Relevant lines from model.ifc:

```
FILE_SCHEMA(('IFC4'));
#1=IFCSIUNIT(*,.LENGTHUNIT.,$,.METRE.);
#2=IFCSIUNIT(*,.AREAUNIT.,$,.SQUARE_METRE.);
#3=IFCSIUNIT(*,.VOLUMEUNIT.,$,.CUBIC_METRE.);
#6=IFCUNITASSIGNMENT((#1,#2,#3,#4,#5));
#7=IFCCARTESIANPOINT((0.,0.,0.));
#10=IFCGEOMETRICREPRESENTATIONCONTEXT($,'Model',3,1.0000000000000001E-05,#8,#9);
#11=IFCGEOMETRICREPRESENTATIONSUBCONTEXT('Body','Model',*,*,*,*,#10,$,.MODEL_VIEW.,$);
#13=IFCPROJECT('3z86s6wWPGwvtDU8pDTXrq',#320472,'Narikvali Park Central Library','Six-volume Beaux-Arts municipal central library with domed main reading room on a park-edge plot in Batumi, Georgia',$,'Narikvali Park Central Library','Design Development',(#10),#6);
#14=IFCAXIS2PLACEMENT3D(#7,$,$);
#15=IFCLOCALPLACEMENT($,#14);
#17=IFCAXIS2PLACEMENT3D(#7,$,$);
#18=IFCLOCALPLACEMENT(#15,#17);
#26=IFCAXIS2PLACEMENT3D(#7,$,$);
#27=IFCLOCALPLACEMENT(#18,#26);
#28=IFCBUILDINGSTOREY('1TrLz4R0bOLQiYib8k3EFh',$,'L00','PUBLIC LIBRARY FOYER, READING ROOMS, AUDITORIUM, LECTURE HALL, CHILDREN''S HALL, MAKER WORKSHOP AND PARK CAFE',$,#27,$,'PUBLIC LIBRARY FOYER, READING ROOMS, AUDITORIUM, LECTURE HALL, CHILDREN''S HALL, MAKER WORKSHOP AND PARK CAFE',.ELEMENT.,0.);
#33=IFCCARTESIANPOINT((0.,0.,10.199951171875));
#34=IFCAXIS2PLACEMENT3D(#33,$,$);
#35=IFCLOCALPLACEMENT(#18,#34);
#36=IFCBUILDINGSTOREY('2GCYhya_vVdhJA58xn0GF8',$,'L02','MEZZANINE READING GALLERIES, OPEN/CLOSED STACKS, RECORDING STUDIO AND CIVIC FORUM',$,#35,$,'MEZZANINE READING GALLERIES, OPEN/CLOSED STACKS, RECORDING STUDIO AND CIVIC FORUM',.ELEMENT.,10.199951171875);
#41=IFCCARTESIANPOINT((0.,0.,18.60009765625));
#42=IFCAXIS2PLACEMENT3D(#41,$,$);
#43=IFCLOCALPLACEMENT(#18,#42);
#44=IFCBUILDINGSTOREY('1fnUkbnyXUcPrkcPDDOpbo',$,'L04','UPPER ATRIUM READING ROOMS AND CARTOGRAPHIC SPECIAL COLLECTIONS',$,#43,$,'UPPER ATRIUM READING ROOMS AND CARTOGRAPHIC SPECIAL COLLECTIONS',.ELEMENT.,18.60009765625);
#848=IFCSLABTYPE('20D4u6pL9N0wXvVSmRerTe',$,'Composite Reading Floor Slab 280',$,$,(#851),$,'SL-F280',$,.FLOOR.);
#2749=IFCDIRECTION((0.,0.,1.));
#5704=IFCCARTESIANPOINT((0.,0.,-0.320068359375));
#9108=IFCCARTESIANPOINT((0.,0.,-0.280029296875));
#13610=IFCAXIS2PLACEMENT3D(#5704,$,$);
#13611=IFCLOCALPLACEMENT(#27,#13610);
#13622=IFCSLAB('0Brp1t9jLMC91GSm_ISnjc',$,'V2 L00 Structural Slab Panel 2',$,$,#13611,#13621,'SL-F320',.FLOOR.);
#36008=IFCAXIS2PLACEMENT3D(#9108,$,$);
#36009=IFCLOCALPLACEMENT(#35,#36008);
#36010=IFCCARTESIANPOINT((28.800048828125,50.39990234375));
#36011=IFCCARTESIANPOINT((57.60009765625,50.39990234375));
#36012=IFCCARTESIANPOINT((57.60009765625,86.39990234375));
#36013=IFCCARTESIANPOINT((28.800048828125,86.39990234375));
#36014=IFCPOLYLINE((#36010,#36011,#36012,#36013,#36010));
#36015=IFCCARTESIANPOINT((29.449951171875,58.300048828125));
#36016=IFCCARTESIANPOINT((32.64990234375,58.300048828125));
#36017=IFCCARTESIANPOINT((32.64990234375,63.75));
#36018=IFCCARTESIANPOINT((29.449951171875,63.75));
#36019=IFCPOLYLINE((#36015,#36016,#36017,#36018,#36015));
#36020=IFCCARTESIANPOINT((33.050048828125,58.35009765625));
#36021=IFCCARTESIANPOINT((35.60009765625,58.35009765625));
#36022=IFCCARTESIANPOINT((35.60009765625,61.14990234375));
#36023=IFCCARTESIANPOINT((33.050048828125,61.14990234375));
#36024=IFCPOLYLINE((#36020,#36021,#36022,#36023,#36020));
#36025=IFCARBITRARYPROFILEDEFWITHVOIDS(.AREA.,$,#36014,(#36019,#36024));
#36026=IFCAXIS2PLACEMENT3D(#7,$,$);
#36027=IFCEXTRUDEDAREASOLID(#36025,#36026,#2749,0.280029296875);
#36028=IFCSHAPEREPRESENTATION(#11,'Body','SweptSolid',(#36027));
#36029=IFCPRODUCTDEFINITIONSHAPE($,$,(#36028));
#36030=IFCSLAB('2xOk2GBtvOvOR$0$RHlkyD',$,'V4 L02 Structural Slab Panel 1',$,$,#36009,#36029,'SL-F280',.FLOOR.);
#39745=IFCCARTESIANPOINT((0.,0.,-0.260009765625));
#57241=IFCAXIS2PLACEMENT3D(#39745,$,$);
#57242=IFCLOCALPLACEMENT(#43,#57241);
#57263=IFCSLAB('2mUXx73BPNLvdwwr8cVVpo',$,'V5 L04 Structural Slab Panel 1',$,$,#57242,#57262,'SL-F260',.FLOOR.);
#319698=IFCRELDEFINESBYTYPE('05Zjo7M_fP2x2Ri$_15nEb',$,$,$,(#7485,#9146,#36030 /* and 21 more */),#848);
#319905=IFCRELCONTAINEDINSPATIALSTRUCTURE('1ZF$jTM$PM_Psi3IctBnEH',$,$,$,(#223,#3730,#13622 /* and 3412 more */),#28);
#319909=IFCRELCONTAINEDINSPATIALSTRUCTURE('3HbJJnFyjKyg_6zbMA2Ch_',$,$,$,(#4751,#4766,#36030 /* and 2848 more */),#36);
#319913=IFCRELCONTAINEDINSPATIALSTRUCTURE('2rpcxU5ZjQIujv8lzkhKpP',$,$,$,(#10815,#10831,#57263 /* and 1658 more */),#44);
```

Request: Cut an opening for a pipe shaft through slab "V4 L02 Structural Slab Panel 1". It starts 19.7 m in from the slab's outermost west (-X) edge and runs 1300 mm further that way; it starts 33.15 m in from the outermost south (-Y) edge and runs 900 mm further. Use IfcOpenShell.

```python
import numpy as np
import ifcopenshell
import ifcopenshell.api.feature
import ifcopenshell.api.geometry
import ifcopenshell.api.root
import ifcopenshell.geom
import ifcopenshell.util.placement
import ifcopenshell.util.representation
import ifcopenshell.util.shape
import ifcopenshell.util.unit

model = ifcopenshell.open("model.ifc")
unit_scale = ifcopenshell.util.unit.calculate_unit_scale(model)
settings = ifcopenshell.geom.settings()


def volume(element):
    """Net volume in cubic metres, openings subtracted."""
    shape = ifcopenshell.geom.create_shape(settings, element)
    return ifcopenshell.util.shape.get_volume(shape.geometry)


slab = model.by_guid("2xOk2GBtvOvOR$0$RHlkyD")
before = volume(slab)

# Extent in the slab's own axes, in metres. The edges named are its -X and -Y sides.
slab_shape = ifcopenshell.geom.create_shape(settings, slab)
vertices = ifcopenshell.util.shape.get_vertices(slab_shape.geometry)
x_min, y_min, bottom = vertices.min(axis=0)
top = vertices[:, 2].max()

opening = ifcopenshell.api.root.create_entity(model, ifc_class="IfcOpeningElement", name="Pipe shaft opening", predefined_type="OPENING")
context = ifcopenshell.util.representation.get_context(model, "Model", "Body", "MODEL_VIEW")
width, depth = 1.3, 0.9
outline = [(0.0, 0.0), (width, 0.0), (width, depth), (0.0, depth), (0.0, 0.0)]
# Overshoot both faces by 50 mm so the cut is clean.
shape = ifcopenshell.api.geometry.add_slab_representation(
    model, context=context, depth=top - bottom + 0.1, polyline=outline
)
ifcopenshell.api.geometry.assign_representation(model, product=opening, representation=shape)

matrix = ifcopenshell.util.placement.get_local_placement(slab.ObjectPlacement)
matrix[:, 3] = matrix @ np.append(np.array([x_min + 19.7, y_min + 33.15, bottom - 0.05]) / unit_scale, 1.0)
ifcopenshell.api.geometry.edit_object_placement(model, product=opening, matrix=matrix, is_si=False)
ifcopenshell.api.feature.add_feature(model, feature=opening, element=slab)

after = volume(slab)

print(f"slab volume {before:.3f} -> {after:.3f} m3")

model.write("model_updated.ifc")
```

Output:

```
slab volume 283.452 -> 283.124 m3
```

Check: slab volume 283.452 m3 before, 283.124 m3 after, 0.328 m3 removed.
